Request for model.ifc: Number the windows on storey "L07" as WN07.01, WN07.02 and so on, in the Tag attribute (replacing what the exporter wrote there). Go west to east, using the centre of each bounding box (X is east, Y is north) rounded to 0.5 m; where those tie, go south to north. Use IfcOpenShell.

First a look at what the model holds.

```python
import ifcopenshell
import ifcopenshell.util.element
import ifcopenshell.util.placement

model = ifcopenshell.open("model.ifc")
print(model.schema)
storey = next(s for s in model.by_type("IfcBuildingStorey") if s.Name == "L07")
windows = [e for e in ifcopenshell.util.element.get_decomposition(storey) if e.is_a("IfcWindow")]
for e in sorted(windows, key=lambda e: e.id()):
    origin = ifcopenshell.util.placement.get_local_placement(e.ObjectPlacement)[:3, 3]
    print(e.id(), e.Tag, e.Name, origin.round(2) + 0.0, sep=" | ")
```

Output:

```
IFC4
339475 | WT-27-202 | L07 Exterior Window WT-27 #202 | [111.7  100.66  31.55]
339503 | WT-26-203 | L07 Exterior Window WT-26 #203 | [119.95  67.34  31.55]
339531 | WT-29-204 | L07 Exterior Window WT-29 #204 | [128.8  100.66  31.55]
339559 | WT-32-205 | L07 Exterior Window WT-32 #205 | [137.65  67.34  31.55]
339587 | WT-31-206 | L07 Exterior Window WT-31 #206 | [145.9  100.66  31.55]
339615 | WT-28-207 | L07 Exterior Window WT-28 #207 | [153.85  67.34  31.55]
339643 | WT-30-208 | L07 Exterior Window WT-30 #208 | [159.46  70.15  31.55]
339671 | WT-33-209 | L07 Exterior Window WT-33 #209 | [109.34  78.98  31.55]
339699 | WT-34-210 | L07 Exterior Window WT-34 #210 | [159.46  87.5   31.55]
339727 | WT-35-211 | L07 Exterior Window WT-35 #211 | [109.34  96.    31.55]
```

```python
import ifcopenshell
import ifcopenshell.geom
import ifcopenshell.util.element
import ifcopenshell.util.shape

model = ifcopenshell.open("model.ifc")
settings = ifcopenshell.geom.settings()
settings.set("use-world-coords", True)


def centre(element):
    shape = ifcopenshell.geom.create_shape(settings, element)
    return ifcopenshell.util.shape.get_bbox_centroid(shape.geometry)


storey = next(s for s in model.by_type("IfcBuildingStorey") if s.Name == "L07")
windows = [e for e in ifcopenshell.util.element.get_decomposition(storey) if e.is_a("IfcWindow")]

# Insertion points can sit at a corner or the storey origin, so sort by the geometry (in metres).
centres = {e: centre(e) for e in windows}
windows.sort(key=lambda e: (round(centres[e][0] / 0.5), centres[e][1]))

for i, e in enumerate(windows, start=1):
    number = f"WN07.{i:02d}"
    e.Tag = number
    print(e.id(), number)

model.write("model_v2.ifc")
```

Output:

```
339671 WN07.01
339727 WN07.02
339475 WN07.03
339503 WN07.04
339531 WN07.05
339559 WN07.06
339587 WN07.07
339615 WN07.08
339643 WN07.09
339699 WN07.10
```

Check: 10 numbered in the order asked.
